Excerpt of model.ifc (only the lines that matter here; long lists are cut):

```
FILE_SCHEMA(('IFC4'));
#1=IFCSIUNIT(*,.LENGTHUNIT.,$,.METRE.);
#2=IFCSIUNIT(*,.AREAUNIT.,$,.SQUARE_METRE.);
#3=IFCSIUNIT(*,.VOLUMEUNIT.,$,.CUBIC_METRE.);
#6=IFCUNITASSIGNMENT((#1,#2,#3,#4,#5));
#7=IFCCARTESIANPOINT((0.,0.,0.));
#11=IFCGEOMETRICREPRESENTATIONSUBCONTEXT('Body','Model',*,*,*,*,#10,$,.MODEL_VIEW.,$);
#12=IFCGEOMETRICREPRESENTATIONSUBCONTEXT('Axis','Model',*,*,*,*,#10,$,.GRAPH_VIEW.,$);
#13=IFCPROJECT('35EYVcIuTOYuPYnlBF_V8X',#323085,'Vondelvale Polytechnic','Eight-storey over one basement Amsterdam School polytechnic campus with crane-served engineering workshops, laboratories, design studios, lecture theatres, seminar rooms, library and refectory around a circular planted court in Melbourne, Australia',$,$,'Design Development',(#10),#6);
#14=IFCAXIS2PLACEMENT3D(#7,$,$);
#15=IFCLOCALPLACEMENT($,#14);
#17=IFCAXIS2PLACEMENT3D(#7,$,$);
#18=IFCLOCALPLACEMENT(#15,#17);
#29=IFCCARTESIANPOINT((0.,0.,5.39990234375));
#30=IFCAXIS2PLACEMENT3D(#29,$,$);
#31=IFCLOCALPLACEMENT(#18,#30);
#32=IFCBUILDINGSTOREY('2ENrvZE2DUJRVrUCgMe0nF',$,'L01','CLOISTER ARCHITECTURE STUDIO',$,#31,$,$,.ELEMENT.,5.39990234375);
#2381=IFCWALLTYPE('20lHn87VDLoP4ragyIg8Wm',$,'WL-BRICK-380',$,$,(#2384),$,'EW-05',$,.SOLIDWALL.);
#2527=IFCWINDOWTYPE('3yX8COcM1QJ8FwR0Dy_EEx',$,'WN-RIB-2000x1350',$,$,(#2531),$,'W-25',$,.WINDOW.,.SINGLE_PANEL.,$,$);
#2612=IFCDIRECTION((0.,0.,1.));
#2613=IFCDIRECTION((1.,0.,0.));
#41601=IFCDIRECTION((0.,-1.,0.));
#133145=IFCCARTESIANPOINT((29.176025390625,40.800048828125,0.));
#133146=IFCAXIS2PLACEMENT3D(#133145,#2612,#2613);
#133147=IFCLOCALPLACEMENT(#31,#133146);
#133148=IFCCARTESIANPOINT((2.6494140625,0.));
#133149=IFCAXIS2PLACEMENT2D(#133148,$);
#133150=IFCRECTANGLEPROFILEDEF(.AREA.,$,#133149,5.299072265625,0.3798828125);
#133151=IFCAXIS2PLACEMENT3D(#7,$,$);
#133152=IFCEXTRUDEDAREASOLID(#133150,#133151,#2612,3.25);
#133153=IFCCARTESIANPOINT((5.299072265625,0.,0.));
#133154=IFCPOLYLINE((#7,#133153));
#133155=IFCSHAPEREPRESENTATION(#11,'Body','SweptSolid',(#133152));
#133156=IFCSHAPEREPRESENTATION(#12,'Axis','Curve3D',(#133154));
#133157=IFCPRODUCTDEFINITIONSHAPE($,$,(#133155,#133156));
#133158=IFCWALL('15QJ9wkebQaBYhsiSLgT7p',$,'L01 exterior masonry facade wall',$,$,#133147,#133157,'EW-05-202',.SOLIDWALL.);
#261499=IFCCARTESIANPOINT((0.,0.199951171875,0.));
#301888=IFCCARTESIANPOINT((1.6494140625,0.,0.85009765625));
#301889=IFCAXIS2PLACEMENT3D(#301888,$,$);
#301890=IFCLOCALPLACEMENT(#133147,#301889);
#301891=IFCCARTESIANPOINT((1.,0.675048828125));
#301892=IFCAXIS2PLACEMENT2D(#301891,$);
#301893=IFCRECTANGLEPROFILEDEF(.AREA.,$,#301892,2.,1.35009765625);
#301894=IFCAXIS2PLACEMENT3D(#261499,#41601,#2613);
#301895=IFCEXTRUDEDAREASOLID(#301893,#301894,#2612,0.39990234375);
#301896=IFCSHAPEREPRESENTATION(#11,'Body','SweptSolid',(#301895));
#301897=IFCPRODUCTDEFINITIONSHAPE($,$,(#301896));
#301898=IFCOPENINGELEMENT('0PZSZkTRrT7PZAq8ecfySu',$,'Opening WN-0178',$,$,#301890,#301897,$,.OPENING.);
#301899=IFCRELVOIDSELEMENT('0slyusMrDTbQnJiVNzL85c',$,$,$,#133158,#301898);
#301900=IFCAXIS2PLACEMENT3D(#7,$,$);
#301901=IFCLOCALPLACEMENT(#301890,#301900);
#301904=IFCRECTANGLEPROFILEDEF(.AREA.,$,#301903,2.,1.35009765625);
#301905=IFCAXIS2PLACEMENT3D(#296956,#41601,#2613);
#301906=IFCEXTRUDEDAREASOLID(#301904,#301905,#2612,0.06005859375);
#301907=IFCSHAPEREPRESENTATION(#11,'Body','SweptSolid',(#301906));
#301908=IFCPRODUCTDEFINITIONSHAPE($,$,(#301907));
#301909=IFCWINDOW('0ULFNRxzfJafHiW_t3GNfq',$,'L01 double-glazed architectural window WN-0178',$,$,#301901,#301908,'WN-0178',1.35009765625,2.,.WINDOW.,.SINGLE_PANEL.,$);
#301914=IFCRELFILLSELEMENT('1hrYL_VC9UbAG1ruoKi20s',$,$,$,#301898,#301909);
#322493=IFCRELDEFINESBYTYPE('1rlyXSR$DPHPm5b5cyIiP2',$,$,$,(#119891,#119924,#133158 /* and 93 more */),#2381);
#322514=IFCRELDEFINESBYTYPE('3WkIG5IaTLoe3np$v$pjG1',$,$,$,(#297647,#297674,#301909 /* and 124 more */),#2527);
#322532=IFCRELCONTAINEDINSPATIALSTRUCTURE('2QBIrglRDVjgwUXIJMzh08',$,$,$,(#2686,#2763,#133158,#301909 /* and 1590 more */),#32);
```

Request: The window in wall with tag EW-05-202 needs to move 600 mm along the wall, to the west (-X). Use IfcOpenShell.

```python
import ifcopenshell
import ifcopenshell.api.geometry
import ifcopenshell.util.placement

model = ifcopenshell.open("model.ifc")

window = model.by_id(301909)
opening = window.FillsVoids[0].RelatingOpeningElement
wall = opening.VoidsElements[0].RelatingBuildingElement

wall_matrix = ifcopenshell.util.placement.get_local_placement(wall.ObjectPlacement)
shift = wall_matrix[:3, 0] * -0.6
before = ifcopenshell.util.placement.get_local_placement(window.ObjectPlacement)[:3, 3].copy()

# The window is placed relative to its opening, so it follows when the opening moves.
matrix = ifcopenshell.util.placement.get_local_placement(opening.ObjectPlacement)
matrix[:3, 3] += shift
ifcopenshell.api.geometry.edit_object_placement(
    model, product=opening, matrix=matrix, is_si=False, should_transform_children=True
)

after = ifcopenshell.util.placement.get_local_placement(window.ObjectPlacement)[:3, 3]
print("window moved by", (after - before).round(3) + 0.0)

model.write("model_v2.ifc")
```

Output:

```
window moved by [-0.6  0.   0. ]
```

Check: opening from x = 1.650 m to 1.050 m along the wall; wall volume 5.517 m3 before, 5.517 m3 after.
